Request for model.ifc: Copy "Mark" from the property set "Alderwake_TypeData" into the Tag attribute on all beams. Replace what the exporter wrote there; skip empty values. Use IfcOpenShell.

First a look at what the model holds.

```python
import ifcopenshell
import ifcopenshell.util.element

model = ifcopenshell.open("model.ifc")
print(model.schema)
beams = model.by_type("IfcBeam")
print(len(beams), "beams")
for e in beams[:8]:
    source = ifcopenshell.util.element.get_pset(e, "Alderwake_TypeData", "Mark")
    target = e.Tag
    print(e.id(), repr(source), repr(target), sep=" | ")
```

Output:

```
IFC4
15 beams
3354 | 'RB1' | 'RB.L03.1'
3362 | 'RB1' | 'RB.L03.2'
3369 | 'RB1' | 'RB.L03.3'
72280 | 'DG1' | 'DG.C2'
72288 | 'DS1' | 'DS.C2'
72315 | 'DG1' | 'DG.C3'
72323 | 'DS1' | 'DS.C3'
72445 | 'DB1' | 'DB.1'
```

```python
import ifcopenshell
import ifcopenshell.util.element

model = ifcopenshell.open("model.ifc")

count = 0
for e in model.by_type("IfcBeam"):
    value = ifcopenshell.util.element.get_pset(e, "Alderwake_TypeData", "Mark")
    current = e.Tag
    if not value or not value.strip() or current == value:
        continue
    e.Tag = value
    count += 1

print(count, "beams updated")

model.write("model_updated.ifc")
```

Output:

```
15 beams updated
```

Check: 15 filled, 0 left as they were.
